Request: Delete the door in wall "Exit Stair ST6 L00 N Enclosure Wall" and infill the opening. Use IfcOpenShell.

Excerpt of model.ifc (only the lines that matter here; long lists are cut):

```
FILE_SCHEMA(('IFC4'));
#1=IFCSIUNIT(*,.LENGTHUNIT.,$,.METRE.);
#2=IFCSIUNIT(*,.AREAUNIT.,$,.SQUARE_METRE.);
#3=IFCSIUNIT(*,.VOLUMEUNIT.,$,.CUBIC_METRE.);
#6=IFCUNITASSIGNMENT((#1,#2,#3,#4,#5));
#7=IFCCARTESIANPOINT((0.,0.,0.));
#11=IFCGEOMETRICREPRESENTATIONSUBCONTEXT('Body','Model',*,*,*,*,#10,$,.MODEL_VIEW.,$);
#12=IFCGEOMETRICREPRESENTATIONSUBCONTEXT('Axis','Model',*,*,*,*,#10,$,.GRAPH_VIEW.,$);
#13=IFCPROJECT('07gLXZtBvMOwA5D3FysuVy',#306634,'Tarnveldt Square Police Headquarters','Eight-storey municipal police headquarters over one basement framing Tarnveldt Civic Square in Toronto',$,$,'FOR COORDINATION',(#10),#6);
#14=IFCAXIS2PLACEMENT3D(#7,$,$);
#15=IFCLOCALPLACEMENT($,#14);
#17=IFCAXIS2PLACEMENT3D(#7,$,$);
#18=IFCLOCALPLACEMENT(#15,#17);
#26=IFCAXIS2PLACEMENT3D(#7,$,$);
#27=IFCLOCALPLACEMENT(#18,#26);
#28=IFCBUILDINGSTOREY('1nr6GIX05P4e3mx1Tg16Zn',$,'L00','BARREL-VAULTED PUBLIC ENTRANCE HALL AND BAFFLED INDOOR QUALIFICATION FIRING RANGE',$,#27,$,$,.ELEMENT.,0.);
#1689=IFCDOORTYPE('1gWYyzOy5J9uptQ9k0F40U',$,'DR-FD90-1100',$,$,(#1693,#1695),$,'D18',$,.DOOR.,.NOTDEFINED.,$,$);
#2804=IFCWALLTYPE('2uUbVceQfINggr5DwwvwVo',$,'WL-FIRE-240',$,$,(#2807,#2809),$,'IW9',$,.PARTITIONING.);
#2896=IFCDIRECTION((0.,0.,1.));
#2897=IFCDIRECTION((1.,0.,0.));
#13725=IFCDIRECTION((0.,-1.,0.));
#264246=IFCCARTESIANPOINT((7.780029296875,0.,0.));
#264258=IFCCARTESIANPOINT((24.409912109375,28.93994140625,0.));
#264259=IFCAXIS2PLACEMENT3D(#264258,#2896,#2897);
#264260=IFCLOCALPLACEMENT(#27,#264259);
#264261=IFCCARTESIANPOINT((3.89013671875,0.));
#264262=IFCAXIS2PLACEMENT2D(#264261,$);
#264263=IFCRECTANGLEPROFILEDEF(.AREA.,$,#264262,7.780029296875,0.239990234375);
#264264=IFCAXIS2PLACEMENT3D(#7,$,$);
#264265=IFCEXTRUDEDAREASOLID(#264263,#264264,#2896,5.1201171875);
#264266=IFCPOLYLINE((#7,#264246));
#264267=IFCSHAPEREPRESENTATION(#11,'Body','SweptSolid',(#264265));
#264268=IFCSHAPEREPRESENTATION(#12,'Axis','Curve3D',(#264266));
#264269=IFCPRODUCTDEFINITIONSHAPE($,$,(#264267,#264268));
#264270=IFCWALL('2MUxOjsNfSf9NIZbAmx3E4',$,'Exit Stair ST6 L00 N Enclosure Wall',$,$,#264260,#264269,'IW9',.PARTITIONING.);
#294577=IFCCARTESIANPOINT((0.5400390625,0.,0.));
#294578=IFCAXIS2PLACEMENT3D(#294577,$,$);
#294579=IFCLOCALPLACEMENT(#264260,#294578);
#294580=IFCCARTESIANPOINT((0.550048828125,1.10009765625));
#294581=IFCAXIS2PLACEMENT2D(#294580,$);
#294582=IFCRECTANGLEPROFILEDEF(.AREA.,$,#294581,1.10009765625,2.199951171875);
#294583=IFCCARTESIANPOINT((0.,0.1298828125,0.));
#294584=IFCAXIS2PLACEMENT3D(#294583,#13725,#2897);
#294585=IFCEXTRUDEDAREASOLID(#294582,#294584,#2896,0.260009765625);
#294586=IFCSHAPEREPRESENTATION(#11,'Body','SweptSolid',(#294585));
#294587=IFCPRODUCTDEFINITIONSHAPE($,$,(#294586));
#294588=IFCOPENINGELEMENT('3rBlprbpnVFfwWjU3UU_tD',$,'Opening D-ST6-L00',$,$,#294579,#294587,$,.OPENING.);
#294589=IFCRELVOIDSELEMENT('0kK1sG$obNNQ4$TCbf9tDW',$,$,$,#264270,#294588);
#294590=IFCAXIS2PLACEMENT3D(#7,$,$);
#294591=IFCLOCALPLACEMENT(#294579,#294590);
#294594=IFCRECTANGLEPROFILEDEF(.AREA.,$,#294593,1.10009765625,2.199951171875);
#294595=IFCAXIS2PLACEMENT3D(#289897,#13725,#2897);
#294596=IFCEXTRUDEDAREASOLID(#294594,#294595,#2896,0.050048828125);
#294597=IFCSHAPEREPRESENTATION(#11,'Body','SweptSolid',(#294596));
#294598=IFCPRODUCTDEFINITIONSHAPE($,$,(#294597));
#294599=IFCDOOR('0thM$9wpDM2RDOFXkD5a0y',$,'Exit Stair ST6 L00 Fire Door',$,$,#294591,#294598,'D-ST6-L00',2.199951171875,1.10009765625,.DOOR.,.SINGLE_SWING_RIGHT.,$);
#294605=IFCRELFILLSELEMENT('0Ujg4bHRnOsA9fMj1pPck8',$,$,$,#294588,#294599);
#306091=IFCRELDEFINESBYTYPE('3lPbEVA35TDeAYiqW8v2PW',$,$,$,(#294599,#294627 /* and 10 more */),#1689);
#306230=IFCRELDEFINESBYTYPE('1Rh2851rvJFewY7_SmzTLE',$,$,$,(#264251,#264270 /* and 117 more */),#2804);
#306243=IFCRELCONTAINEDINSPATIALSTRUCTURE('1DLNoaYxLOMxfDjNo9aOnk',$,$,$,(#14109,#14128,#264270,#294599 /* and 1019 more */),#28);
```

```python
import ifcopenshell
import ifcopenshell.api.feature
import ifcopenshell.api.root
import ifcopenshell.geom
import ifcopenshell.util.shape

model = ifcopenshell.open("model.ifc")
settings = ifcopenshell.geom.settings()


def volume(element):
    """Net volume in cubic metres, openings subtracted."""
    shape = ifcopenshell.geom.create_shape(settings, element)
    return ifcopenshell.util.shape.get_volume(shape.geometry)


door = model.by_guid("0thM$9wpDM2RDOFXkD5a0y")
opening = door.FillsVoids[0].RelatingOpeningElement
wall = opening.VoidsElements[0].RelatingBuildingElement
before = volume(wall)

ifcopenshell.api.root.remove_product(model, product=door)
ifcopenshell.api.feature.remove_feature(model, feature=opening)

after = volume(wall)

print(f"wall volume {before:.3f} -> {after:.3f} m3")

model.write("model_edited.ifc")
```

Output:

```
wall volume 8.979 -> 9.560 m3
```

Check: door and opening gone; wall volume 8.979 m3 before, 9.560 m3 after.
